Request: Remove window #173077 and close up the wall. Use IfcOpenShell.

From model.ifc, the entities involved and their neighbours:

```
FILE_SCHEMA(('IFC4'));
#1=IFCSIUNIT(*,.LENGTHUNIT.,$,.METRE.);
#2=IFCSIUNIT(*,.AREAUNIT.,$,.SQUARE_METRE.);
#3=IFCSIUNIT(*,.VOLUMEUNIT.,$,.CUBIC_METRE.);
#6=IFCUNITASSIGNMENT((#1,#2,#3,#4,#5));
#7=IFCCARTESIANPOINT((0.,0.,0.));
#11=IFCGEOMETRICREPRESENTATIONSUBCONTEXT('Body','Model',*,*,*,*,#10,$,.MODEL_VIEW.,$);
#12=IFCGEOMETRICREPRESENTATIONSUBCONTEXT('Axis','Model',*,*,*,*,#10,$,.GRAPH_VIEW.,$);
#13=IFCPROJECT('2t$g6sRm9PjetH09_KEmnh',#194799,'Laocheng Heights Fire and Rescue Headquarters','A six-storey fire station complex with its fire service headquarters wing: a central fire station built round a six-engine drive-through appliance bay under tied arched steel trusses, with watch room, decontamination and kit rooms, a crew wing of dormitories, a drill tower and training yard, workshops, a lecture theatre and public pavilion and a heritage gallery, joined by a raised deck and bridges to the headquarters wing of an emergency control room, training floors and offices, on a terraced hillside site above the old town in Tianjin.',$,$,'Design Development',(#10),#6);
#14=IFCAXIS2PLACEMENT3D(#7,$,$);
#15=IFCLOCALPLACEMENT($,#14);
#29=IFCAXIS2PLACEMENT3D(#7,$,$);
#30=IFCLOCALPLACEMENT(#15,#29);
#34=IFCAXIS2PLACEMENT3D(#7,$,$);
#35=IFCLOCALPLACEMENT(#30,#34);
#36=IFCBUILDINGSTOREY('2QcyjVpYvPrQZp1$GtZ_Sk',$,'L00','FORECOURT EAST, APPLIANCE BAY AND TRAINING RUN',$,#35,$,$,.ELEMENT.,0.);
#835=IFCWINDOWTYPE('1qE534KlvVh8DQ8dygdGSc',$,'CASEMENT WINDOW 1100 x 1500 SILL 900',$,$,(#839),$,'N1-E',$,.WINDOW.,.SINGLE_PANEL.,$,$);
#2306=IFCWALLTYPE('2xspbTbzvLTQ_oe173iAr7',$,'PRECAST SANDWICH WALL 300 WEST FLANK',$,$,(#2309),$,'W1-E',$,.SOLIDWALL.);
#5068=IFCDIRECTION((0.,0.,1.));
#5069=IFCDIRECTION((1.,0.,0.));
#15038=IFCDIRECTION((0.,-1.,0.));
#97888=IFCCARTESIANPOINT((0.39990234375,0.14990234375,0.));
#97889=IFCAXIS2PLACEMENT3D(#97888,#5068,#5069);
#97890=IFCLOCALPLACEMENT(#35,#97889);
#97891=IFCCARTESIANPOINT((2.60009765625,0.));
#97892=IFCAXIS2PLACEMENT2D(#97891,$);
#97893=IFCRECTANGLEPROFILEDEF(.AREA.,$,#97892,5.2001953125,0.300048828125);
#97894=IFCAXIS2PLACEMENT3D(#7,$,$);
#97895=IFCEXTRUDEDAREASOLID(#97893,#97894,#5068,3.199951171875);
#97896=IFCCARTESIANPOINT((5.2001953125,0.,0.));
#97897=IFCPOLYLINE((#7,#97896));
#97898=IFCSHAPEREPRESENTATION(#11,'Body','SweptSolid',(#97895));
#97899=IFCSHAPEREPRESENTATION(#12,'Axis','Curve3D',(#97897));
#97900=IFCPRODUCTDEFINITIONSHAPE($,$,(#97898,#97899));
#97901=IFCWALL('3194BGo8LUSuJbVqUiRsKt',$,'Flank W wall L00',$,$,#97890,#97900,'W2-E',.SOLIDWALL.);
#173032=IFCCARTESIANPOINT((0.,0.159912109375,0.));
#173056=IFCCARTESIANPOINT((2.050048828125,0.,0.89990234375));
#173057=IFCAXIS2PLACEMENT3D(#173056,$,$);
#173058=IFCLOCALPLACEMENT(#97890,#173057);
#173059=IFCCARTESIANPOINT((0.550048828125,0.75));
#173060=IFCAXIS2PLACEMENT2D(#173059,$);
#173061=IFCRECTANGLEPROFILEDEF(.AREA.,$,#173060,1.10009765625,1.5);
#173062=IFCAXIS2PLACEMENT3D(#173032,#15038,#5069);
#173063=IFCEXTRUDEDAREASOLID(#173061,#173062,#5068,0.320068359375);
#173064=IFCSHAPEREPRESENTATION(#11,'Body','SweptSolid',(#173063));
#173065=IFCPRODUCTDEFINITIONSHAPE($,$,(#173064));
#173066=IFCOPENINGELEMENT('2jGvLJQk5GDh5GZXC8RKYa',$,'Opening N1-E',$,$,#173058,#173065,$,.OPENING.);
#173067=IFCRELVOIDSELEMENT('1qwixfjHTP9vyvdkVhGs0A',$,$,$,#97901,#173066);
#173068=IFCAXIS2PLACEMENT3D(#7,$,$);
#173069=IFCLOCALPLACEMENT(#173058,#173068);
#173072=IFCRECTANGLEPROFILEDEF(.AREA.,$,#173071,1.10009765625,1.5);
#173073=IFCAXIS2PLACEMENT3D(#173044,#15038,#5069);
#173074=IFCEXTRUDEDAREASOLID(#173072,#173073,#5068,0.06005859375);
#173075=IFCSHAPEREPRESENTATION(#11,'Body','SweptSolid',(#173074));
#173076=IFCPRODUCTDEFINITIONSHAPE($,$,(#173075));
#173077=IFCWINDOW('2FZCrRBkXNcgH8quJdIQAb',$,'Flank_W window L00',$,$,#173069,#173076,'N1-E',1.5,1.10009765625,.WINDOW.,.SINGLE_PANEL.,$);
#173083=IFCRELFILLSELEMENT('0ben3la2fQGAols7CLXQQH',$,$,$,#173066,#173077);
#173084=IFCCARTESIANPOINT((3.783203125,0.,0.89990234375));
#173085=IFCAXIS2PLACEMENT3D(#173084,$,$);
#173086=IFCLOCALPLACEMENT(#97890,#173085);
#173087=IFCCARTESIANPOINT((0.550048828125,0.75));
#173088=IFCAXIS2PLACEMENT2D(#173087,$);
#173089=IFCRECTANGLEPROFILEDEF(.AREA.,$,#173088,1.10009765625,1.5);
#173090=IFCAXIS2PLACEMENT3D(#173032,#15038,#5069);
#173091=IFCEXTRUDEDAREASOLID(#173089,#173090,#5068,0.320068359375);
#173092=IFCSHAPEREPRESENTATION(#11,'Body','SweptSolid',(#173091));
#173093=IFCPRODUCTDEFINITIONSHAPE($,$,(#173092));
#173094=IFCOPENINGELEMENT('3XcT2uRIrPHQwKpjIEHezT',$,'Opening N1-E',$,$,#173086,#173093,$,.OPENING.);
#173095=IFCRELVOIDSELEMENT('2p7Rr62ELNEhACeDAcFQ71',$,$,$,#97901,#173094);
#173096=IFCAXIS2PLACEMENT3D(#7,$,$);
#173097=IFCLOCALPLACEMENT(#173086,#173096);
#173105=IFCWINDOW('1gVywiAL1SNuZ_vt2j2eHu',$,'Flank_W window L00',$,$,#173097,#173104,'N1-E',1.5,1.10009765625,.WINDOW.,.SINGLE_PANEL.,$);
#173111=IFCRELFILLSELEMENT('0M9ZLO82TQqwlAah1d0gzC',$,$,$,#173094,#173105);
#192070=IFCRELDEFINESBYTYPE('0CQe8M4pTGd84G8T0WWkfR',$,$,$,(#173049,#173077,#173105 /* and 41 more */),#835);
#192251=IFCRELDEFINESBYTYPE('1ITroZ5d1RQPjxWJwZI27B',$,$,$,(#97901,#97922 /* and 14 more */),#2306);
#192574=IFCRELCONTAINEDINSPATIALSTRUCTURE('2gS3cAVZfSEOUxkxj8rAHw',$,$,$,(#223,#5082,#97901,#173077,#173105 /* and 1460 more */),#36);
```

```python
import ifcopenshell
import ifcopenshell.api.feature
import ifcopenshell.api.root
import ifcopenshell.geom
import ifcopenshell.util.shape

model = ifcopenshell.open("model.ifc")
settings = ifcopenshell.geom.settings()


def volume(element):
    """Net volume in cubic metres, openings subtracted."""
    shape = ifcopenshell.geom.create_shape(settings, element)
    return ifcopenshell.util.shape.get_volume(shape.geometry)


window = model.by_guid("2FZCrRBkXNcgH8quJdIQAb")
opening = window.FillsVoids[0].RelatingOpeningElement
wall = opening.VoidsElements[0].RelatingBuildingElement
before = volume(wall)

ifcopenshell.api.root.remove_product(model, product=window)
ifcopenshell.api.feature.remove_feature(model, feature=opening)

after = volume(wall)

print(f"wall volume {before:.3f} -> {after:.3f} m3")

model.write("model_rev.ifc")
```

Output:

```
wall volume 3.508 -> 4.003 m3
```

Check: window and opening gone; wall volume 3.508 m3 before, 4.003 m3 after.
